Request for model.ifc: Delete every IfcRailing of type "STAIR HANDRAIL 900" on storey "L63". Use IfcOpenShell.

First a look at what the model holds.

```python
import ifcopenshell
import ifcopenshell.util.element

model = ifcopenshell.open("model.ifc")
print(model.schema)
storey = next(s for s in model.by_type("IfcBuildingStorey") if s.Name == "L63")
railings = [e for e in ifcopenshell.util.element.get_decomposition(storey) if e.is_a("IfcRailing")]
seen = {}
for e in railings:
    element_type = ifcopenshell.util.element.get_type(e)
    name = element_type.Name if element_type not in (None, e) else None
    seen[name] = seen.get(name, 0) + 1
for name, count in sorted(seen.items(), key=str):
    print(count, "x", name)
```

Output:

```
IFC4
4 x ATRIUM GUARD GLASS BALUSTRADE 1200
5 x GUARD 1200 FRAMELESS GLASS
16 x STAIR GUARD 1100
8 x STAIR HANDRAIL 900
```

```python
import ifcopenshell
import ifcopenshell.api.root
import ifcopenshell.util.element

model = ifcopenshell.open("model.ifc")

storey = next(s for s in model.by_type("IfcBuildingStorey") if s.Name == "L63")
railings = [e for e in ifcopenshell.util.element.get_decomposition(storey) if e.is_a("IfcRailing")]
targets = [e for e in railings if (t := ifcopenshell.util.element.get_type(e)) not in (None, e) and t.Name == "STAIR HANDRAIL 900"]

for e in targets:
    ifcopenshell.api.root.remove_product(model, product=e)
print(len(targets), "removed")

model.write("model_updated.ifc")
```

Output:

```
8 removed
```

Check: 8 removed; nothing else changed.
